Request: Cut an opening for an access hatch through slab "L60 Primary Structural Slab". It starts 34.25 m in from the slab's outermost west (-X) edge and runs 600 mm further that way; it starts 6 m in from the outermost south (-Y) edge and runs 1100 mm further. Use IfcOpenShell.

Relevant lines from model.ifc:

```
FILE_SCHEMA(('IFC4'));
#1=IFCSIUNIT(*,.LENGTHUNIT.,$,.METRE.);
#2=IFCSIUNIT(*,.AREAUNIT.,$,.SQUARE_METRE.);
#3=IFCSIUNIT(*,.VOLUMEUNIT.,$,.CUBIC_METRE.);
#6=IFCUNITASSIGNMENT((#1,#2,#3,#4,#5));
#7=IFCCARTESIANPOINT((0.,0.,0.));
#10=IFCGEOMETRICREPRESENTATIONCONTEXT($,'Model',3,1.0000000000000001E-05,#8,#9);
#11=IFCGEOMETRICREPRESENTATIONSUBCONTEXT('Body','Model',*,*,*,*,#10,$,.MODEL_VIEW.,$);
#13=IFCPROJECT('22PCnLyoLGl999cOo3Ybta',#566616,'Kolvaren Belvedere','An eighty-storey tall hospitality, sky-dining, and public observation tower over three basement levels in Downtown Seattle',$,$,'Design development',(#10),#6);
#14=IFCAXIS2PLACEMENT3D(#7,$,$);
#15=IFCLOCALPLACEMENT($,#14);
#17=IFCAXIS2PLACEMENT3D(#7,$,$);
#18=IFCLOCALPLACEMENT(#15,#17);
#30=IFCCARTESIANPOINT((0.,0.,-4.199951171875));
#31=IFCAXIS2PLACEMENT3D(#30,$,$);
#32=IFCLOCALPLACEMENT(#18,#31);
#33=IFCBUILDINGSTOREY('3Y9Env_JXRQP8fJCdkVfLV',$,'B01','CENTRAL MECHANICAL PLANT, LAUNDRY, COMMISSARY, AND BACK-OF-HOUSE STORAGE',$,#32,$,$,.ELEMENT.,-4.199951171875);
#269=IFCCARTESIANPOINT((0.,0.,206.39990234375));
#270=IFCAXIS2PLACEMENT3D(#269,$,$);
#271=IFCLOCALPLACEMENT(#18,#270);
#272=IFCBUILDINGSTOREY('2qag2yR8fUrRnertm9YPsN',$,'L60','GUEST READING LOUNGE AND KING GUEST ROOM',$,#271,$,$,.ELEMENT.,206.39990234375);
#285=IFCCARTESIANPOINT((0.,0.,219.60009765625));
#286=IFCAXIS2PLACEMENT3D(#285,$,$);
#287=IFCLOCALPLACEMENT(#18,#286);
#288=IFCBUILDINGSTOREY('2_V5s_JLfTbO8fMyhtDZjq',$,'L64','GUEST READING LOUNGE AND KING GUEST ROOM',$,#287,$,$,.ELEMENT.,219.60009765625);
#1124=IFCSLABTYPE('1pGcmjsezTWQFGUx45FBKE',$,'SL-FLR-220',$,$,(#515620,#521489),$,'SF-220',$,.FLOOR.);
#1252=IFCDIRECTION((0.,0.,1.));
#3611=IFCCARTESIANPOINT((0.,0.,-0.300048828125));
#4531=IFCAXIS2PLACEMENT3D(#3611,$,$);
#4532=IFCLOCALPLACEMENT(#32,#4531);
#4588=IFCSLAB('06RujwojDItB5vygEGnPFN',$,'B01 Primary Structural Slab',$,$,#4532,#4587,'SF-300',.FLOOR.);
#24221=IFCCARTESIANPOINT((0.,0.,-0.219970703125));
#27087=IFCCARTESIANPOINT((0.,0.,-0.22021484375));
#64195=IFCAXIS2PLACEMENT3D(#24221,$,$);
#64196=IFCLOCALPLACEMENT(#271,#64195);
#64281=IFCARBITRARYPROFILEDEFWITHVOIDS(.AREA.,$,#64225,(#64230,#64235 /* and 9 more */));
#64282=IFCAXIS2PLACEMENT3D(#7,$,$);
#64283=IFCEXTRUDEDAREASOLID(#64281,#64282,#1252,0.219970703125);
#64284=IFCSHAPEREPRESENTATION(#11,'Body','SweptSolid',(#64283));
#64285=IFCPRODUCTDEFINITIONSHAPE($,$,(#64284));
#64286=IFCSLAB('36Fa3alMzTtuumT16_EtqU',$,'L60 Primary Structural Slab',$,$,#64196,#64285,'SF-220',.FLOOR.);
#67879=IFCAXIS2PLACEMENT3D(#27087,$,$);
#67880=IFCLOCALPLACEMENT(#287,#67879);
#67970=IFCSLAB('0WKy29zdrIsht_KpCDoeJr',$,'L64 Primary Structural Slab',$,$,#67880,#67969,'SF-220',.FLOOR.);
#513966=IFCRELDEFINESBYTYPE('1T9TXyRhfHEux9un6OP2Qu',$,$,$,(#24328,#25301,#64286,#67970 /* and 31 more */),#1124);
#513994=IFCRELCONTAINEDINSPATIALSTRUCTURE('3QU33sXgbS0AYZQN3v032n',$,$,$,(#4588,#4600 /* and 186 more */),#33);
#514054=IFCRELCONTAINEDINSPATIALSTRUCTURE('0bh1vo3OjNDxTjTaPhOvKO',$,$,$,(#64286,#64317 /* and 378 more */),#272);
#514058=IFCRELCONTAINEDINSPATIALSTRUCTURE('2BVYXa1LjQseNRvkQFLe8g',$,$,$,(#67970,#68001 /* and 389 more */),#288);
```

```python
import numpy as np
import ifcopenshell
import ifcopenshell.api.feature
import ifcopenshell.api.geometry
import ifcopenshell.api.root
import ifcopenshell.geom
import ifcopenshell.util.placement
import ifcopenshell.util.representation
import ifcopenshell.util.shape
import ifcopenshell.util.unit

model = ifcopenshell.open("model.ifc")
unit_scale = ifcopenshell.util.unit.calculate_unit_scale(model)
settings = ifcopenshell.geom.settings()


def volume(element):
    """Net volume in cubic metres, openings subtracted."""
    shape = ifcopenshell.geom.create_shape(settings, element)
    return ifcopenshell.util.shape.get_volume(shape.geometry)


slab = model.by_id(64286)
before = volume(slab)

# Extent in the slab's own axes, in metres. The edges named are its -X and -Y sides.
slab_shape = ifcopenshell.geom.create_shape(settings, slab)
vertices = ifcopenshell.util.shape.get_vertices(slab_shape.geometry)
x_min, y_min, bottom = vertices.min(axis=0)
top = vertices[:, 2].max()

opening = ifcopenshell.api.root.create_entity(model, ifc_class="IfcOpeningElement", name="Access hatch opening", predefined_type="OPENING")
context = ifcopenshell.util.representation.get_context(model, "Model", "Body", "MODEL_VIEW")
width, depth = 0.6, 1.1
outline = [(0.0, 0.0), (width, 0.0), (width, depth), (0.0, depth), (0.0, 0.0)]
# Overshoot both faces by 50 mm so the cut is clean.
shape = ifcopenshell.api.geometry.add_slab_representation(
    model, context=context, depth=top - bottom + 0.1, polyline=outline
)
ifcopenshell.api.geometry.assign_representation(model, product=opening, representation=shape)

matrix = ifcopenshell.util.placement.get_local_placement(slab.ObjectPlacement)
matrix[:, 3] = matrix @ np.append(np.array([x_min + 34.25, y_min + 6, bottom - 0.05]) / unit_scale, 1.0)
ifcopenshell.api.geometry.edit_object_placement(model, product=opening, matrix=matrix, is_si=False)
ifcopenshell.api.feature.add_feature(model, feature=opening, element=slab)

after = volume(slab)

print(f"slab volume {before:.3f} -> {after:.3f} m3")

model.write("model_rev.ifc")
```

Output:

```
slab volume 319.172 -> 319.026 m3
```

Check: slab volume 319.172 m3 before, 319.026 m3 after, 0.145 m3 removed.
